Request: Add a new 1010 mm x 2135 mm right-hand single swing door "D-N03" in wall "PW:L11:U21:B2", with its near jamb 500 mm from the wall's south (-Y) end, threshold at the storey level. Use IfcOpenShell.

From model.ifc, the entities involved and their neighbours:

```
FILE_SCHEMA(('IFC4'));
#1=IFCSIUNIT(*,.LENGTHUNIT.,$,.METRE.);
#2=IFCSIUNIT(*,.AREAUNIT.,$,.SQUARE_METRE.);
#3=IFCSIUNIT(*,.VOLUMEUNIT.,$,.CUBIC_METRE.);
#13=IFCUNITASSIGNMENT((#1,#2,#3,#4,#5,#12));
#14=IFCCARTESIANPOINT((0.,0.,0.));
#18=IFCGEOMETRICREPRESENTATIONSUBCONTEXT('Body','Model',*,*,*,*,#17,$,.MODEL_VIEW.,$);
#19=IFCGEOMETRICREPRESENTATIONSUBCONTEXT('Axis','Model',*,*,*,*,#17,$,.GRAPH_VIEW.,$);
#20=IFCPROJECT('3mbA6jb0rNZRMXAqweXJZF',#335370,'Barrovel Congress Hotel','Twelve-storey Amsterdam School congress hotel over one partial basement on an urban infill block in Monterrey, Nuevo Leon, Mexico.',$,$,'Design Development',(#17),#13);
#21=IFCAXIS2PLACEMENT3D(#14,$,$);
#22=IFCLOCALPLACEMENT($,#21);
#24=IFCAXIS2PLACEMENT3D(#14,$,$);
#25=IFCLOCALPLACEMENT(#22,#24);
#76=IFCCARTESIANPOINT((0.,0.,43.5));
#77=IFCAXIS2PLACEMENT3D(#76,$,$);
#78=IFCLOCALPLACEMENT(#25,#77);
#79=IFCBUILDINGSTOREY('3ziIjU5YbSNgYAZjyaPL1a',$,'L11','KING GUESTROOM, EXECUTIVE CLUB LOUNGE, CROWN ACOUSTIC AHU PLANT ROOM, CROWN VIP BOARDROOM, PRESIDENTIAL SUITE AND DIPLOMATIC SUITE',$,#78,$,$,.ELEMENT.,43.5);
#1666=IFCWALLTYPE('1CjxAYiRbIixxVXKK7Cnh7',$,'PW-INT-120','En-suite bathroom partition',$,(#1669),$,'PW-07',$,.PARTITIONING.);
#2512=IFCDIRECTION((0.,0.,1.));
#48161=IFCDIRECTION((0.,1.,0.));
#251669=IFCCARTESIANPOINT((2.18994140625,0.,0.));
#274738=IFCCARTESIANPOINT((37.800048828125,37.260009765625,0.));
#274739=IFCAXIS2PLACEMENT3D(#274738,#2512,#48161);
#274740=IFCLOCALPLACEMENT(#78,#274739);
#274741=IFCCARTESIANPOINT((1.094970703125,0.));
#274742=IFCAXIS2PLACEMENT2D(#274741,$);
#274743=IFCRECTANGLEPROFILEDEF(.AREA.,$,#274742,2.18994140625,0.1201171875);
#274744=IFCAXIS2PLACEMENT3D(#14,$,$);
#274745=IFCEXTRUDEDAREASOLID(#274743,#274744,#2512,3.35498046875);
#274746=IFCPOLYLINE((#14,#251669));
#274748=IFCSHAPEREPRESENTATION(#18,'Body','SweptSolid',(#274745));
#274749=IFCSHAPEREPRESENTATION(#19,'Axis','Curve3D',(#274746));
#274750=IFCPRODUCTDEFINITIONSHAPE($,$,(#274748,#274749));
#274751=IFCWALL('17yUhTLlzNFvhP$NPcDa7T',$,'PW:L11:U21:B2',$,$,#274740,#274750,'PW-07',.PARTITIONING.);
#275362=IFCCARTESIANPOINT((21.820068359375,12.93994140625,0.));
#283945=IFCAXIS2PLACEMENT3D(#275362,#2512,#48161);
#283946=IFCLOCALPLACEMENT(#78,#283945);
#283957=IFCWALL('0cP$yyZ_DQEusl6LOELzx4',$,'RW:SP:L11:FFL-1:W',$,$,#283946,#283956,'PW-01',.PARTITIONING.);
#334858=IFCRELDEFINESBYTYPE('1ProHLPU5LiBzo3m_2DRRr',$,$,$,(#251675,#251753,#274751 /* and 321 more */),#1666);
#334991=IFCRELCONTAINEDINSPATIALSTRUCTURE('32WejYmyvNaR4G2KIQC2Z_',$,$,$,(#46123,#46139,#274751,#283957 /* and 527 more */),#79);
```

```python
import numpy as np
import ifcopenshell
import ifcopenshell.api.feature
import ifcopenshell.api.geometry
import ifcopenshell.api.root
import ifcopenshell.api.spatial
import ifcopenshell.geom
import ifcopenshell.util.element
import ifcopenshell.util.placement
import ifcopenshell.util.representation
import ifcopenshell.util.shape
import ifcopenshell.util.unit

model = ifcopenshell.open("model.ifc")
unit_scale = ifcopenshell.util.unit.calculate_unit_scale(model)
settings = ifcopenshell.geom.settings()


def volume(element):
    """Net volume in cubic metres, openings subtracted."""
    shape = ifcopenshell.geom.create_shape(settings, element)
    return ifcopenshell.util.shape.get_volume(shape.geometry)


wall = model.by_guid("17yUhTLlzNFvhP$NPcDa7T")
storey = ifcopenshell.util.element.get_container(wall, ifc_class="IfcBuildingStorey")
context = ifcopenshell.util.representation.get_context(model, "Model", "Body", "MODEL_VIEW")
before = volume(wall)

width, height, from_end, sill = 1.01, 2.135, 0.5, 0.0  # metres

# The wall runs along its own X axis, and the end named is its -X end.
wall_shape = ifcopenshell.geom.create_shape(settings, wall)
x, y, z = ifcopenshell.util.shape.get_vertices(wall_shape.geometry).T
start = x.min() + from_end
face, thickness = float(y.min()), float(y.max() - y.min())
wall_matrix = ifcopenshell.util.placement.get_local_placement(wall.ObjectPlacement)
level = ifcopenshell.util.placement.get_local_placement(storey.ObjectPlacement)[2, 3]


def in_wall(x, y):
    """Placement at x, y metres in the wall's axes, at sill height."""
    matrix = wall_matrix.copy()
    matrix[:, 3] = wall_matrix @ np.array([x / unit_scale, y / unit_scale, 0.0, 1.0])
    matrix[2, 3] = level + sill / unit_scale
    return matrix


# Opening: a box that overshoots both wall faces by 50 mm.
opening = ifcopenshell.api.root.create_entity(model, ifc_class="IfcOpeningElement", predefined_type="OPENING")
box = ifcopenshell.api.geometry.add_wall_representation(
    model, context=context, length=width, height=height, thickness=thickness + 0.1
)
ifcopenshell.api.geometry.assign_representation(model, product=opening, representation=box)
ifcopenshell.api.geometry.edit_object_placement(model, product=opening, matrix=in_wall(start, face - 0.05), is_si=False)
ifcopenshell.api.feature.add_feature(model, feature=opening, element=wall)

door = ifcopenshell.api.root.create_entity(model, ifc_class="IfcDoor", name="D-N03", predefined_type="DOOR")
door.OverallWidth, door.OverallHeight = width / unit_scale, height / unit_scale
door.OperationType = "SINGLE_SWING_RIGHT"
body = ifcopenshell.api.geometry.add_door_representation(
    model,
    context=context,
    overall_width=door.OverallWidth,
    overall_height=door.OverallHeight,
    operation_type="SINGLE_SWING_RIGHT",
    lining_properties={"LiningDepth": thickness / unit_scale, "ThresholdDepth": thickness / unit_scale},
)
ifcopenshell.api.geometry.assign_representation(model, product=door, representation=body)
ifcopenshell.api.spatial.assign_container(model, products=[door], relating_structure=storey)
ifcopenshell.api.feature.add_filling(model, opening=opening, element=door)

# The lining spans the wall, so the door starts at the wall face.
ifcopenshell.api.geometry.edit_object_placement(model, product=door, matrix=in_wall(start, face), is_si=False)

after = volume(wall)

print(f"wall volume {before:.3f} -> {after:.3f} m3")

model.write("model_updated.ifc")
```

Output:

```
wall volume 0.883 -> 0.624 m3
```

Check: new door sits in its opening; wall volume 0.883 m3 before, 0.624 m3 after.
